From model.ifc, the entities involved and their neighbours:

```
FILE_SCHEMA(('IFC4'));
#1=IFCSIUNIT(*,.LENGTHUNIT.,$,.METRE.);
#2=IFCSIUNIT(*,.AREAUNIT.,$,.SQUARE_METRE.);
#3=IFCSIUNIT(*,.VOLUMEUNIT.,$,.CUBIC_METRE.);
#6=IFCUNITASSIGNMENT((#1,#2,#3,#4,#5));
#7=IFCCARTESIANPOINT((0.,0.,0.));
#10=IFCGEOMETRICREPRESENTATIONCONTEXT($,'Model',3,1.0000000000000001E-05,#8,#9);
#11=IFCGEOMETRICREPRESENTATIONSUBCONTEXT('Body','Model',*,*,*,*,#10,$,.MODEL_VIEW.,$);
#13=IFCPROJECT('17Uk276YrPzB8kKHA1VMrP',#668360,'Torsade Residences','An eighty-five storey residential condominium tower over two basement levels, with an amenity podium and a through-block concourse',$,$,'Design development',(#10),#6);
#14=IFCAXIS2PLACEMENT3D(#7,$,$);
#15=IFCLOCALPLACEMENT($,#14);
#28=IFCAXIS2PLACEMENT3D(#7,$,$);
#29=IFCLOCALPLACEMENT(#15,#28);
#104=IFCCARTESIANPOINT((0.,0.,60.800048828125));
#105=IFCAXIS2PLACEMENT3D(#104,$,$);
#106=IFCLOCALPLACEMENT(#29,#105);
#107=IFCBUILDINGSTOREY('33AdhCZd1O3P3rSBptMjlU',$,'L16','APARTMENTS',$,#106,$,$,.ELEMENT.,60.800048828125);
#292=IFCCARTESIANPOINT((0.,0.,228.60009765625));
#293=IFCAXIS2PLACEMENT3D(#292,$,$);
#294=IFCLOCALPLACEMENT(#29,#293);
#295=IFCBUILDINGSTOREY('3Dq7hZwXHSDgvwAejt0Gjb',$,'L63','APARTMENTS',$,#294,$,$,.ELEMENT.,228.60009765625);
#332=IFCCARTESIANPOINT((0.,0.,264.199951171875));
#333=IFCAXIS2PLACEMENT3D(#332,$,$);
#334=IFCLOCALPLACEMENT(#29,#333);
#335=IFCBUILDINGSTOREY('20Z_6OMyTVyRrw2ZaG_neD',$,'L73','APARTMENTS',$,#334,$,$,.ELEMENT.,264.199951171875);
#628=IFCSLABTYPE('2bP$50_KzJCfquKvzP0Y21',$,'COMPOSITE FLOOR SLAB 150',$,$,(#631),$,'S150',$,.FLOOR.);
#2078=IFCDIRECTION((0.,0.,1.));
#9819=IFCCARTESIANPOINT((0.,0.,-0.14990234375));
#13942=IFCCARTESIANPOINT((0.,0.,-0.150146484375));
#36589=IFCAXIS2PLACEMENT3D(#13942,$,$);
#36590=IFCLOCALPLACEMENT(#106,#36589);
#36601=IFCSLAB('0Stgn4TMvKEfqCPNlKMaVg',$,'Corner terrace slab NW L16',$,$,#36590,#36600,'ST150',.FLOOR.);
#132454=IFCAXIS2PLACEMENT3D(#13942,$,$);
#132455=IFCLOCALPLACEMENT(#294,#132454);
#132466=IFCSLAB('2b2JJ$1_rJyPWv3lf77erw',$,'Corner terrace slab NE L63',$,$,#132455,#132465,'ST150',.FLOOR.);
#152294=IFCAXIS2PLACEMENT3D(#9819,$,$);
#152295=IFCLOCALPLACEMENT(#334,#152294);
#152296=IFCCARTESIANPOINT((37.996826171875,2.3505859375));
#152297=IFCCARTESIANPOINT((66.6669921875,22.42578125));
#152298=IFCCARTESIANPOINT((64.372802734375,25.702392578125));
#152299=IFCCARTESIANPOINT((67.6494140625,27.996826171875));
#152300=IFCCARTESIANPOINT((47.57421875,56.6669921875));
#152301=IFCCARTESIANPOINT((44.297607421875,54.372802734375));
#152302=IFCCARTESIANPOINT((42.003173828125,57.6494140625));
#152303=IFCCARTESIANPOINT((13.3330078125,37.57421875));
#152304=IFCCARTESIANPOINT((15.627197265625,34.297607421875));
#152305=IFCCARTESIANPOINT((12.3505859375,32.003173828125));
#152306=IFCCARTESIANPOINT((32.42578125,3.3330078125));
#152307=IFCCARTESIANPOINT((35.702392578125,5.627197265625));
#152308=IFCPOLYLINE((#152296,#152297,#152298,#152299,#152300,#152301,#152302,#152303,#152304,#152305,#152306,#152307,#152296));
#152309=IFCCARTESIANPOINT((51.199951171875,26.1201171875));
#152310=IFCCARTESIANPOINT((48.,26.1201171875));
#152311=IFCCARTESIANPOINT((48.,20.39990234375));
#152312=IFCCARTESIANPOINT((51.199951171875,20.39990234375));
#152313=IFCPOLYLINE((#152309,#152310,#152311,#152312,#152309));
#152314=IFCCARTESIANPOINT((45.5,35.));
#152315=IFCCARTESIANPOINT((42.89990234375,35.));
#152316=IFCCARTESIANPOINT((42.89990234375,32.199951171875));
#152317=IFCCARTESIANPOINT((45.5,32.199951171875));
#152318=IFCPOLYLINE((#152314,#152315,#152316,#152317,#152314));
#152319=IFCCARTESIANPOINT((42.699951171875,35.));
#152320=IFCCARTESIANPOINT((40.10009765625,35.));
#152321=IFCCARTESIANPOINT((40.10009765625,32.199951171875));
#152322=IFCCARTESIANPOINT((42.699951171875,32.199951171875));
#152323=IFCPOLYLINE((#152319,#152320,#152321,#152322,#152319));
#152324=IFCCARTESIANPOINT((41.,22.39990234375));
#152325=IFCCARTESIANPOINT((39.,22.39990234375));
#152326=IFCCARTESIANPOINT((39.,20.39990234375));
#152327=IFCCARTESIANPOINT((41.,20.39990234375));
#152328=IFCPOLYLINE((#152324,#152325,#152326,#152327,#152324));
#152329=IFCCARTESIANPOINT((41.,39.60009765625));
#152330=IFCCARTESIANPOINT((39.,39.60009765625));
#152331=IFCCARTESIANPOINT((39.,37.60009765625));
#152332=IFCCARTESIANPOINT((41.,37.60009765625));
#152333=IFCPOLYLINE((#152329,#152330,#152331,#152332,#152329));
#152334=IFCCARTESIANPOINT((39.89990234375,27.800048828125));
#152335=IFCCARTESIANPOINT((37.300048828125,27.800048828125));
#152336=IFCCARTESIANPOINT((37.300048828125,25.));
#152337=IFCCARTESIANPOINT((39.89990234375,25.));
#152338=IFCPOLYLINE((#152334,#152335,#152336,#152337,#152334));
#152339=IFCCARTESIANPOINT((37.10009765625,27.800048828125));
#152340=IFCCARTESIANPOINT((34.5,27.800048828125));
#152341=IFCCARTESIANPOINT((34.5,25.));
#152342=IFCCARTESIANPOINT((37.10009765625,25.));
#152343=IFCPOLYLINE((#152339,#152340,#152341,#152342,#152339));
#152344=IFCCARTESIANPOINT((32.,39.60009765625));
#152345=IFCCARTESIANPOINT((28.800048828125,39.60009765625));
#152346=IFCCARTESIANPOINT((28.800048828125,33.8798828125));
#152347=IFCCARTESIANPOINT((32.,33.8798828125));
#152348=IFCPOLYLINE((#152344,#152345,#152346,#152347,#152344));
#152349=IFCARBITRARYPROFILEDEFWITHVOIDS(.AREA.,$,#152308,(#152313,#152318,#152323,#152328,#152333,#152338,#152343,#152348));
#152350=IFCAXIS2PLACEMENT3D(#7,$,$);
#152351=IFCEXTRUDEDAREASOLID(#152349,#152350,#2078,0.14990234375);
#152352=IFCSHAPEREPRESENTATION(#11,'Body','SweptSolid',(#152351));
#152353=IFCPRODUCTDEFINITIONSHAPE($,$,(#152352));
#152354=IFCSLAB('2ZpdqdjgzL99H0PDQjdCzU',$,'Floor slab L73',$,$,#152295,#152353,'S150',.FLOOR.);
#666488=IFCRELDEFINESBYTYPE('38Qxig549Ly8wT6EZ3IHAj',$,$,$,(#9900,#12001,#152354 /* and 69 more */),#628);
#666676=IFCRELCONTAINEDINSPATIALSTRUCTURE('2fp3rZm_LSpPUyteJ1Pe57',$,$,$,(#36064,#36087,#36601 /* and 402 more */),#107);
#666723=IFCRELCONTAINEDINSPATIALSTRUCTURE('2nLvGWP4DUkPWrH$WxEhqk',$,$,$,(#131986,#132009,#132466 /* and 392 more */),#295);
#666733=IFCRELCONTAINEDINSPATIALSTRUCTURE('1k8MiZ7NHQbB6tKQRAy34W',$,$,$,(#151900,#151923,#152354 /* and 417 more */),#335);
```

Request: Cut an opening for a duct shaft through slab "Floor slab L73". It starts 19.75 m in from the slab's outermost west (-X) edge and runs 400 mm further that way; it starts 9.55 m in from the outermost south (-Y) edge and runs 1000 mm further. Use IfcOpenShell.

```python
import numpy as np
import ifcopenshell
import ifcopenshell.api.feature
import ifcopenshell.api.geometry
import ifcopenshell.api.root
import ifcopenshell.geom
import ifcopenshell.util.placement
import ifcopenshell.util.representation
import ifcopenshell.util.shape
import ifcopenshell.util.unit

model = ifcopenshell.open("model.ifc")
unit_scale = ifcopenshell.util.unit.calculate_unit_scale(model)
settings = ifcopenshell.geom.settings()


def volume(element):
    """Net volume in cubic metres, openings subtracted."""
    shape = ifcopenshell.geom.create_shape(settings, element)
    return ifcopenshell.util.shape.get_volume(shape.geometry)


slab = model.by_guid("2ZpdqdjgzL99H0PDQjdCzU")
before = volume(slab)

# Extent in the slab's own axes, in metres. The edges named are its -X and -Y sides.
slab_shape = ifcopenshell.geom.create_shape(settings, slab)
vertices = ifcopenshell.util.shape.get_vertices(slab_shape.geometry)
x_min, y_min, bottom = vertices.min(axis=0)
top = vertices[:, 2].max()

opening = ifcopenshell.api.root.create_entity(model, ifc_class="IfcOpeningElement", name="Duct shaft opening", predefined_type="OPENING")
context = ifcopenshell.util.representation.get_context(model, "Model", "Body", "MODEL_VIEW")
width, depth = 0.4, 1
outline = [(0.0, 0.0), (width, 0.0), (width, depth), (0.0, depth), (0.0, 0.0)]
# Overshoot both faces by 50 mm so the cut is clean.
shape = ifcopenshell.api.geometry.add_slab_representation(
    model, context=context, depth=top - bottom + 0.1, polyline=outline
)
ifcopenshell.api.geometry.assign_representation(model, product=opening, representation=shape)

matrix = ifcopenshell.util.placement.get_local_placement(slab.ObjectPlacement)
matrix[:, 3] = matrix @ np.append(np.array([x_min + 19.75, y_min + 9.55, bottom - 0.05]) / unit_scale, 1.0)
ifcopenshell.api.geometry.edit_object_placement(model, product=opening, matrix=matrix, is_si=False)
ifcopenshell.api.feature.add_feature(model, feature=opening, element=slab)

after = volume(slab)

print(f"slab volume {before:.3f} -> {after:.3f} m3")

model.write("model_v2.ifc")
```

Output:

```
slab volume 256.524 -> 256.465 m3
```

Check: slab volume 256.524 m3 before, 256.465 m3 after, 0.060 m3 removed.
